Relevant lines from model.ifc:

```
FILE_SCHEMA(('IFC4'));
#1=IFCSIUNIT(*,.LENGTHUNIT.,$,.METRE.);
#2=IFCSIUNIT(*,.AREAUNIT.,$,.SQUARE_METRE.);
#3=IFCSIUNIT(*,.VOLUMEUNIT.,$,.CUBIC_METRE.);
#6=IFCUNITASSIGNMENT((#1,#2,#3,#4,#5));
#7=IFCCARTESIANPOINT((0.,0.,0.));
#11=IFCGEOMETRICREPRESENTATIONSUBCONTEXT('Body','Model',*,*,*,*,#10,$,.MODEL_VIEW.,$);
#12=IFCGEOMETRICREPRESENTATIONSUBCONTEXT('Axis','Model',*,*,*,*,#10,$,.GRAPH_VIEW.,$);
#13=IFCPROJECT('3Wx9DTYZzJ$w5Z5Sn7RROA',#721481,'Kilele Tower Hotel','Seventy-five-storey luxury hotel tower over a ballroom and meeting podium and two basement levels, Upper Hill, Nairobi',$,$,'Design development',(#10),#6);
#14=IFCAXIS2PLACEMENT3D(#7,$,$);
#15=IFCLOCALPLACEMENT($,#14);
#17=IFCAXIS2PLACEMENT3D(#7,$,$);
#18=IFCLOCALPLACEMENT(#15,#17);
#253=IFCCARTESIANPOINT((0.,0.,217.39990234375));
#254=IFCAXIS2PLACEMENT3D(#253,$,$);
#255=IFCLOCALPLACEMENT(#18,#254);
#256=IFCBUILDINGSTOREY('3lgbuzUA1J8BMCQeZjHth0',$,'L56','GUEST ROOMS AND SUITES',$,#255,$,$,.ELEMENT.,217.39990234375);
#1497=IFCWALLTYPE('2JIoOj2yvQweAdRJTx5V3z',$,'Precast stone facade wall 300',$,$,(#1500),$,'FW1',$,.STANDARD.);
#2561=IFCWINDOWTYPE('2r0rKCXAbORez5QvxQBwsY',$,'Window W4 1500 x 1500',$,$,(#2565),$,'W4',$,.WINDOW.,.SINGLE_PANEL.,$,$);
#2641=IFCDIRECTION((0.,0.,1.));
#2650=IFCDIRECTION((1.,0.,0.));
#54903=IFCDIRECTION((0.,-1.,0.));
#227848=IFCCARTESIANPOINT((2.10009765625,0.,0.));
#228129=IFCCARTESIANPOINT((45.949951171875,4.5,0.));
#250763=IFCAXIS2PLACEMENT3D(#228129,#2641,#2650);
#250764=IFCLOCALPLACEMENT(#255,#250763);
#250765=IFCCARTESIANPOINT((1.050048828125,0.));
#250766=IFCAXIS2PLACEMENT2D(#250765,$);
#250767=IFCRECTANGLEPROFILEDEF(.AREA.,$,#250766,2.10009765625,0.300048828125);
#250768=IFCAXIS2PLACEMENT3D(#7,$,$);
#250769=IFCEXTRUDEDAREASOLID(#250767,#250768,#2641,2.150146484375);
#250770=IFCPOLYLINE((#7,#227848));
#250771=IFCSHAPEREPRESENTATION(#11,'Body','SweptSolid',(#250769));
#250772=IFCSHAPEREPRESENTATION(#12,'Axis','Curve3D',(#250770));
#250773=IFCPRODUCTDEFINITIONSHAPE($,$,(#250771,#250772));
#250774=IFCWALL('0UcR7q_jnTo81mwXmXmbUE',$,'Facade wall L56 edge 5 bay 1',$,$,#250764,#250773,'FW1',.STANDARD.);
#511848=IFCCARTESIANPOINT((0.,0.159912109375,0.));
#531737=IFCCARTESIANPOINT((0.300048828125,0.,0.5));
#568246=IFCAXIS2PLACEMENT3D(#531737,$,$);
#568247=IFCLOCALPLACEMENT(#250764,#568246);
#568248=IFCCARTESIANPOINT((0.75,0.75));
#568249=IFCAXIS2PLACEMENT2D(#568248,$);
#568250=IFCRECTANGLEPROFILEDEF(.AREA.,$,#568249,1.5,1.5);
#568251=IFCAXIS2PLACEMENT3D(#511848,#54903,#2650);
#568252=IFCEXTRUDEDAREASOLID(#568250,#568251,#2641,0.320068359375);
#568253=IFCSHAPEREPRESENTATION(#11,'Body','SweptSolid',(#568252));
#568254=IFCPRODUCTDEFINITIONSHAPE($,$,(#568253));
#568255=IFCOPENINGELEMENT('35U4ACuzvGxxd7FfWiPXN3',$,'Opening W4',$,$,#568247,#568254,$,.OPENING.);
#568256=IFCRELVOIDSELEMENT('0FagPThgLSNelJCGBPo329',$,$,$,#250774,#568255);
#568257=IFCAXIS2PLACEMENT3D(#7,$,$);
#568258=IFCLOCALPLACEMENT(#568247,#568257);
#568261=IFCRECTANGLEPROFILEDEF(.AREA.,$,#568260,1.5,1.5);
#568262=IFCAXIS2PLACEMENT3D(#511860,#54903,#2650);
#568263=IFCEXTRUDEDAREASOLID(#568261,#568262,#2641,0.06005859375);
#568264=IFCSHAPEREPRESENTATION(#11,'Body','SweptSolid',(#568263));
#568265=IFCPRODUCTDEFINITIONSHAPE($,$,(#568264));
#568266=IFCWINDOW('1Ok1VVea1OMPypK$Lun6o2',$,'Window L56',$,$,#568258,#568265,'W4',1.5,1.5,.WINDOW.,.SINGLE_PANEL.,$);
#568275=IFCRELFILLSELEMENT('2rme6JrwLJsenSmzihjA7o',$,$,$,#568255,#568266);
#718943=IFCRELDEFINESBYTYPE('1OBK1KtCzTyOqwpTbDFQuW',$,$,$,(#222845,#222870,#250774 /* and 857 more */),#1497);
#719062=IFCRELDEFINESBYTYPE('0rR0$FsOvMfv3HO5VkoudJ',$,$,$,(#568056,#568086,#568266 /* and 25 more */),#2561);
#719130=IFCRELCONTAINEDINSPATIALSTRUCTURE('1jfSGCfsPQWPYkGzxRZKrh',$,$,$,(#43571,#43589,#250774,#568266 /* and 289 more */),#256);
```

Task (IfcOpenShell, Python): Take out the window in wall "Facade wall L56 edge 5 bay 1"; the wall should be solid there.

```python
import ifcopenshell
import ifcopenshell.api.feature
import ifcopenshell.api.root
import ifcopenshell.geom
import ifcopenshell.util.shape

model = ifcopenshell.open("model.ifc")
settings = ifcopenshell.geom.settings()


def volume(element):
    """Net volume in cubic metres, openings subtracted."""
    shape = ifcopenshell.geom.create_shape(settings, element)
    return ifcopenshell.util.shape.get_volume(shape.geometry)


window = model.by_id(568266)
opening = window.FillsVoids[0].RelatingOpeningElement
wall = opening.VoidsElements[0].RelatingBuildingElement
before = volume(wall)

ifcopenshell.api.root.remove_product(model, product=window)
ifcopenshell.api.feature.remove_feature(model, feature=opening)

after = volume(wall)

print(f"wall volume {before:.3f} -> {after:.3f} m3")

model.write("model_rev.ifc")
```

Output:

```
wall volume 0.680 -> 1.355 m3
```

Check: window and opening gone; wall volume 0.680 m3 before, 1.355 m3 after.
